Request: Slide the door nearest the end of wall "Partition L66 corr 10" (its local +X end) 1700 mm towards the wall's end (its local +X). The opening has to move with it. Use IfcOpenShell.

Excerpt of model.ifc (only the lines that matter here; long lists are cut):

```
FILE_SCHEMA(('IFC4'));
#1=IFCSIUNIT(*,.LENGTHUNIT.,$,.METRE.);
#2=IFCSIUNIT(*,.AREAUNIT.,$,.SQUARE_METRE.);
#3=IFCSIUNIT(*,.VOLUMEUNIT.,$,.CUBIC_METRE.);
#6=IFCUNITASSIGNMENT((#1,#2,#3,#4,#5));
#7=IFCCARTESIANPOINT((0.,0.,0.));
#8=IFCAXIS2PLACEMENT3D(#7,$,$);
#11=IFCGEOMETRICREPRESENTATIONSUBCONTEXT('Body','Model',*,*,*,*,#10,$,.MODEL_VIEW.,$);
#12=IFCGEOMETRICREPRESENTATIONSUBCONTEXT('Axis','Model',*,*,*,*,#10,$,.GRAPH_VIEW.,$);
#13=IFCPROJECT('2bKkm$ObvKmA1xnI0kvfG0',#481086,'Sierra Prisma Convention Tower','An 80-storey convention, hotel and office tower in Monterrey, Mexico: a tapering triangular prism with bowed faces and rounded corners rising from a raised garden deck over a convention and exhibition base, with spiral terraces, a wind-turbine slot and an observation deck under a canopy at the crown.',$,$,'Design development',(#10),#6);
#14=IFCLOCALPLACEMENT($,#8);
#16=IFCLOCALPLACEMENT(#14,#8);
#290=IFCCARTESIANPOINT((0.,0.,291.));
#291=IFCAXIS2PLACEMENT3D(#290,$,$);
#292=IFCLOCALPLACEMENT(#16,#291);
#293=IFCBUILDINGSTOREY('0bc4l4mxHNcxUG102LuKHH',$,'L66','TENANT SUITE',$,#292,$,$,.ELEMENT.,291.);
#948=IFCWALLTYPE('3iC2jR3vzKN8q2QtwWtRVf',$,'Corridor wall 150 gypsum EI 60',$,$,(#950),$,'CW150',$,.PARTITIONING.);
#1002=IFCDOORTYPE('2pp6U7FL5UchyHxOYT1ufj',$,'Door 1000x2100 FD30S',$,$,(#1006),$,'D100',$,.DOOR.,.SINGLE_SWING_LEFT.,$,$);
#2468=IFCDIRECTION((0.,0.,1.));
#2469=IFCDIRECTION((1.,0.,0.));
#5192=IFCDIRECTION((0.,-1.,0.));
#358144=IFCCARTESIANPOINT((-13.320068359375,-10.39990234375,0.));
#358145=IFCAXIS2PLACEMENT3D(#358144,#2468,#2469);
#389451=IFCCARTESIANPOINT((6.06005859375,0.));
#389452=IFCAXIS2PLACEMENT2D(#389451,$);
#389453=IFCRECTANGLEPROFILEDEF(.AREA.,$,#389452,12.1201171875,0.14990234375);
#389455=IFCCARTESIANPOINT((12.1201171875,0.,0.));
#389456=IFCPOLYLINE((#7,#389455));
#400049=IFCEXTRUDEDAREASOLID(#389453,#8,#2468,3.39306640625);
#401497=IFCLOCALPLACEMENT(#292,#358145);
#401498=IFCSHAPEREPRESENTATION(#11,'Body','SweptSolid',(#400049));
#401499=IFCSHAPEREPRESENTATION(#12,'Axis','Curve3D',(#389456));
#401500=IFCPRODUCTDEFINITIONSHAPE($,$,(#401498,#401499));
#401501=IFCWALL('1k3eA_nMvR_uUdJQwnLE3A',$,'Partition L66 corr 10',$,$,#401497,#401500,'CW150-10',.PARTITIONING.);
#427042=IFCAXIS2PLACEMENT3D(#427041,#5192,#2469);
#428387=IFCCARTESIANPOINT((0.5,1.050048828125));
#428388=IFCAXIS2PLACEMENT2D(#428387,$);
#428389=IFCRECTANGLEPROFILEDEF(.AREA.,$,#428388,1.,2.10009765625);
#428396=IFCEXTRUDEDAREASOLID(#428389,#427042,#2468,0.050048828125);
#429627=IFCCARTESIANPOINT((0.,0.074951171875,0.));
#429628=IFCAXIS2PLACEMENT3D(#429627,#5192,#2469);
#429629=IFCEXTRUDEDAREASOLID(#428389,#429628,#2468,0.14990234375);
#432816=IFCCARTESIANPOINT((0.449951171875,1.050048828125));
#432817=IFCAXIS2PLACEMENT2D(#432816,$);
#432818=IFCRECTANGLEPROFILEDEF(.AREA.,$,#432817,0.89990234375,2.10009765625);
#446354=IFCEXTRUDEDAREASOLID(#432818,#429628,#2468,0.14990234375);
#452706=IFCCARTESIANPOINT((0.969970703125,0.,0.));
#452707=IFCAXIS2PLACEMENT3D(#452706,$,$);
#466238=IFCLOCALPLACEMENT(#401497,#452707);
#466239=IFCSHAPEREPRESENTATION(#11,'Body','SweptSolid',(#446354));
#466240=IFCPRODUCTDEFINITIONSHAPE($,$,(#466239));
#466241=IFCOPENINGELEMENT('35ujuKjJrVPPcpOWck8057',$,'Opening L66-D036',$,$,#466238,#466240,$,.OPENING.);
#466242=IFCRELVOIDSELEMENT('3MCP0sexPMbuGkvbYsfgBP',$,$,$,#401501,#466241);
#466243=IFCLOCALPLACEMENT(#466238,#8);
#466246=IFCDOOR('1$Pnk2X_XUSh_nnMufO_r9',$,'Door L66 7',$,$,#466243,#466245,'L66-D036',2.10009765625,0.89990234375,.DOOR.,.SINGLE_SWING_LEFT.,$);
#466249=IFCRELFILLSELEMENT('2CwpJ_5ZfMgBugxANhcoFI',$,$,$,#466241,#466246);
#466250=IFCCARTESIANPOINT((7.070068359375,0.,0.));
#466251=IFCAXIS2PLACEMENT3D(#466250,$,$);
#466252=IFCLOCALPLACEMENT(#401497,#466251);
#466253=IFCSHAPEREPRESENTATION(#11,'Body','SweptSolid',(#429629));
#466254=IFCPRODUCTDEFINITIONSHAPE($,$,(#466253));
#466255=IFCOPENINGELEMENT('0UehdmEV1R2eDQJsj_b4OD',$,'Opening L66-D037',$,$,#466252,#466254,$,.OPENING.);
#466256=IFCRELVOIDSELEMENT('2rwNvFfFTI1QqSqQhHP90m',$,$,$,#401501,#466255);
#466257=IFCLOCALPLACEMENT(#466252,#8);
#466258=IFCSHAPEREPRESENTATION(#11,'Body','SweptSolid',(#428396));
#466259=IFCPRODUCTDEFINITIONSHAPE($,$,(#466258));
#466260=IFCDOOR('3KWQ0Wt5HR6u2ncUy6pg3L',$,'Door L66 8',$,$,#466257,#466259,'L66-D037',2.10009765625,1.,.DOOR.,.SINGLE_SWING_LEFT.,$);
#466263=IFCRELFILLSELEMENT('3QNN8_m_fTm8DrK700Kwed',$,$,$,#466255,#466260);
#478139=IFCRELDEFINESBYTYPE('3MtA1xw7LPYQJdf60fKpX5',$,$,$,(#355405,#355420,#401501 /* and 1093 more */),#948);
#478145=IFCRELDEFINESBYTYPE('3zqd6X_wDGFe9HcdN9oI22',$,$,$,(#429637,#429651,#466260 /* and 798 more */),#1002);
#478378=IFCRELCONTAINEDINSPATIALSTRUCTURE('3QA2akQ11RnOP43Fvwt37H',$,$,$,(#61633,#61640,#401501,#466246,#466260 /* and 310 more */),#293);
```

```python
import ifcopenshell
import ifcopenshell.api.geometry
import ifcopenshell.util.placement
import ifcopenshell.util.unit

model = ifcopenshell.open("model.ifc")
unit_scale = ifcopenshell.util.unit.calculate_unit_scale(model)

door = model.by_guid("3KWQ0Wt5HR6u2ncUy6pg3L")
opening = door.FillsVoids[0].RelatingOpeningElement
wall = opening.VoidsElements[0].RelatingBuildingElement

wall_matrix = ifcopenshell.util.placement.get_local_placement(wall.ObjectPlacement)
shift = wall_matrix[:3, 0] * 1.7 / unit_scale
before = ifcopenshell.util.placement.get_local_placement(door.ObjectPlacement)[:3, 3].copy()

# The door is placed relative to its opening, so it follows when the opening moves.
matrix = ifcopenshell.util.placement.get_local_placement(opening.ObjectPlacement)
matrix[:3, 3] += shift
ifcopenshell.api.geometry.edit_object_placement(
    model, product=opening, matrix=matrix, is_si=False, should_transform_children=True
)

after = ifcopenshell.util.placement.get_local_placement(door.ObjectPlacement)[:3, 3]
print("door moved by", (after - before).round(3) + 0.0)

model.write("model-out.ifc")
```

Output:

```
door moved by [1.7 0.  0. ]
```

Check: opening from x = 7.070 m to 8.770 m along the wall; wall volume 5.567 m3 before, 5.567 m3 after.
